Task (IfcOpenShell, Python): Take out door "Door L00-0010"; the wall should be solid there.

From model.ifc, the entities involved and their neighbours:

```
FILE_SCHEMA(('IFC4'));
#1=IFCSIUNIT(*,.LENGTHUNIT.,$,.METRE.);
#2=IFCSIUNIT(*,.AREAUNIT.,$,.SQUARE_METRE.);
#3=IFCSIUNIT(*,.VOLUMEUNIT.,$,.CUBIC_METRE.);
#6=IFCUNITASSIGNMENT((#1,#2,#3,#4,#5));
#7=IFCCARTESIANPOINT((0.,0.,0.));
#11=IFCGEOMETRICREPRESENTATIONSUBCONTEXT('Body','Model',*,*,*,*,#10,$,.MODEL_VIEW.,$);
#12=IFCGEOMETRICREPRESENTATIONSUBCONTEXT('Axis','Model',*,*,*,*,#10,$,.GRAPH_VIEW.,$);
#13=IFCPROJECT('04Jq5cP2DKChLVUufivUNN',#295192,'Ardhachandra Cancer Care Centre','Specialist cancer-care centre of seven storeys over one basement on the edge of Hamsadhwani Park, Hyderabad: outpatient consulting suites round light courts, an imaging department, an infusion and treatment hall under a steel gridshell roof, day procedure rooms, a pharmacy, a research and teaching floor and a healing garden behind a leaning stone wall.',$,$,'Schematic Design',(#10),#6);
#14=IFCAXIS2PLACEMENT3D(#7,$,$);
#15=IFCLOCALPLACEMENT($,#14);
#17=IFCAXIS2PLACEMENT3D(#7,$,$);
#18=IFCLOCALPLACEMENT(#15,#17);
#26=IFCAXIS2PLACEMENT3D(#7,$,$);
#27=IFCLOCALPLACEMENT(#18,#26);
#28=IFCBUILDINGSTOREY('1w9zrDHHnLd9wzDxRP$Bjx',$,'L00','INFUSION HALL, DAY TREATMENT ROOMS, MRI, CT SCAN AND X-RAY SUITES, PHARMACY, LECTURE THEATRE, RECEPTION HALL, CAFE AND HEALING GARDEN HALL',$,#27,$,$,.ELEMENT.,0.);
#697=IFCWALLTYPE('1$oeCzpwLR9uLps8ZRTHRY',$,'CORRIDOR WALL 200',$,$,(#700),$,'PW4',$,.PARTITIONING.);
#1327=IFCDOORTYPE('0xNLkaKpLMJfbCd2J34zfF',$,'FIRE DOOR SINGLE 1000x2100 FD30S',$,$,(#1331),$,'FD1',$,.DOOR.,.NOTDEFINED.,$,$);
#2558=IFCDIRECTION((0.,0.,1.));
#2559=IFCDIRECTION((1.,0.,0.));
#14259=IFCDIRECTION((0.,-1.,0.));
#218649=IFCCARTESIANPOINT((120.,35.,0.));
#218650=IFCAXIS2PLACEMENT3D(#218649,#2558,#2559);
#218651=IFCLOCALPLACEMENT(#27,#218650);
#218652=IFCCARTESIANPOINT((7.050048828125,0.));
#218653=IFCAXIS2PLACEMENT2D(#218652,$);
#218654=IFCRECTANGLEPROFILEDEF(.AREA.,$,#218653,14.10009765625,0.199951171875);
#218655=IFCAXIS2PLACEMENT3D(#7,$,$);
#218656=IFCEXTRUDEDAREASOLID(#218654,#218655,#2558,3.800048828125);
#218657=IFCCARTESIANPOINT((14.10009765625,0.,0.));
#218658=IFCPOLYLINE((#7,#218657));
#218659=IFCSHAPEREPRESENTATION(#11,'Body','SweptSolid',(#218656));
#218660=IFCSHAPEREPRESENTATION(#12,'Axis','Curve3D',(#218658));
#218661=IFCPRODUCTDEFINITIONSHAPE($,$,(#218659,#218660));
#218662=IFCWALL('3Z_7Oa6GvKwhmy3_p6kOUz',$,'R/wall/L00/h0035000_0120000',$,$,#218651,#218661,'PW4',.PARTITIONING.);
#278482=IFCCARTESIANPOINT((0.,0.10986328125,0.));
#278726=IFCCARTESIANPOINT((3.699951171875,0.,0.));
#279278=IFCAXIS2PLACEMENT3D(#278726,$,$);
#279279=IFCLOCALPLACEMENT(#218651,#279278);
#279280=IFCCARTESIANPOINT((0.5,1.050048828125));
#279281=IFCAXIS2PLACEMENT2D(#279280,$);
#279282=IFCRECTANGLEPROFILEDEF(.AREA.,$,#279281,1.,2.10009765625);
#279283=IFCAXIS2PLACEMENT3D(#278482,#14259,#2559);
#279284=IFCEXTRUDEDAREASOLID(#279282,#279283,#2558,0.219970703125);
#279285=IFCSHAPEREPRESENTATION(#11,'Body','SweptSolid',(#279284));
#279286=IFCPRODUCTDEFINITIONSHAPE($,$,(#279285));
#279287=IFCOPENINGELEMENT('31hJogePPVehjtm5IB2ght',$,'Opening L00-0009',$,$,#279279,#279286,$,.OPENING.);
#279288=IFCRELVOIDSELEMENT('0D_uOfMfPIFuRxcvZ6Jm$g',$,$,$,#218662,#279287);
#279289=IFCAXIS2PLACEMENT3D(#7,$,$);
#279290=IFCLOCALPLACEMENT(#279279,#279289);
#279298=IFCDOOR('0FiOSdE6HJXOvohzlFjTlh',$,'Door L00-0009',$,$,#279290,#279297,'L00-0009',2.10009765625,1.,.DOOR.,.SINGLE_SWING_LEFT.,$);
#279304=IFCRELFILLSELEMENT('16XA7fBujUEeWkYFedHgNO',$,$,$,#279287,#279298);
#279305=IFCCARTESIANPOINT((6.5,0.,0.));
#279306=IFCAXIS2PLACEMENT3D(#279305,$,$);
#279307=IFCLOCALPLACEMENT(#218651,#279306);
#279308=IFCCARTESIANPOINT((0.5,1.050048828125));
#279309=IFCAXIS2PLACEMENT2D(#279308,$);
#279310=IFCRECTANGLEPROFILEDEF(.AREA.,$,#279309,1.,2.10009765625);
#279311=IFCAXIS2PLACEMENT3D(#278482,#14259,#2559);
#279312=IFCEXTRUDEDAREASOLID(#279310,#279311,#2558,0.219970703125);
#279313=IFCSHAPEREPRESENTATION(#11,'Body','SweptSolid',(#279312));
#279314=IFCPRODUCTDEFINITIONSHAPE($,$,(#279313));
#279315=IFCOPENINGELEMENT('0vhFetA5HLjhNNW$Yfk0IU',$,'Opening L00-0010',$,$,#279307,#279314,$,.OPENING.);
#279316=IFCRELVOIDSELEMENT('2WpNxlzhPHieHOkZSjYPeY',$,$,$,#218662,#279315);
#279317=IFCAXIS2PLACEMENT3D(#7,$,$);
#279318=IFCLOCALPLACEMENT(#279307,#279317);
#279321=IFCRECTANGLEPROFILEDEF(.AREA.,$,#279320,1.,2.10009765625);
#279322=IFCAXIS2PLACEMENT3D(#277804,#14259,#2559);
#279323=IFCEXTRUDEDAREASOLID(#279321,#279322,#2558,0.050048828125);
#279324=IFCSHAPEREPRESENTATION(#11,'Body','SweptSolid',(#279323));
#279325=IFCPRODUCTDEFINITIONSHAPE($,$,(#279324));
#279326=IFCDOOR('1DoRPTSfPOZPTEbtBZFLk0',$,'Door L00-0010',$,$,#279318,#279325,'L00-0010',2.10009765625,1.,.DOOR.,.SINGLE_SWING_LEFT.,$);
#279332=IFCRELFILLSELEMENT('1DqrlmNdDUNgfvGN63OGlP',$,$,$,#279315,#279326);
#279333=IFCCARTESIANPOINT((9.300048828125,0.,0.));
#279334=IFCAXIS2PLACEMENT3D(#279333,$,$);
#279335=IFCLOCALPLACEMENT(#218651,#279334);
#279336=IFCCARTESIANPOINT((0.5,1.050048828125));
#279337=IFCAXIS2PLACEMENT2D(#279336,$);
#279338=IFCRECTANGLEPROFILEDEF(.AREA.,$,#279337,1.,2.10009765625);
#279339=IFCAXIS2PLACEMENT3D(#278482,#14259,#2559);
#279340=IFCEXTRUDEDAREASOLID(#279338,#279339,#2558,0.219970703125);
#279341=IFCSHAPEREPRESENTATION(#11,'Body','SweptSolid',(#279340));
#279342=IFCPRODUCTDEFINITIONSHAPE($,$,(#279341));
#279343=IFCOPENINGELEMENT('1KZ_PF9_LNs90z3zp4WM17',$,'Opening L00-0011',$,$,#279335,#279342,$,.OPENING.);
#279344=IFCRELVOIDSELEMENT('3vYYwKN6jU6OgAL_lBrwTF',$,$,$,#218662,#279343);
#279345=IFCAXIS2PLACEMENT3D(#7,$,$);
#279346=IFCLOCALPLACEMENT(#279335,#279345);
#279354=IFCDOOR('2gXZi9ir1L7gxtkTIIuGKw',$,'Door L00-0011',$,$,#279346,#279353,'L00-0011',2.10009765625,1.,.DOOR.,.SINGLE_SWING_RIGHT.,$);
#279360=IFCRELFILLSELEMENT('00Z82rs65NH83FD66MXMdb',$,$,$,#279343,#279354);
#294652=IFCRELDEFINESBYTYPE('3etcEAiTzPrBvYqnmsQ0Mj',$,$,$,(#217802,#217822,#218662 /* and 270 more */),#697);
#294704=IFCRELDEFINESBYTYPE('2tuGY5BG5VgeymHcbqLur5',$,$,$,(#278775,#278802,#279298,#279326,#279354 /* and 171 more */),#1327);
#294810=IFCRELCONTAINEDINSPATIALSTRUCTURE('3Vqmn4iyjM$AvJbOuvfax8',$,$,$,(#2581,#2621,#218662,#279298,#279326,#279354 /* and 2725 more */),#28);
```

```python
import ifcopenshell
import ifcopenshell.api.feature
import ifcopenshell.api.root
import ifcopenshell.geom
import ifcopenshell.util.shape

model = ifcopenshell.open("model.ifc")
settings = ifcopenshell.geom.settings()


def volume(element):
    """Net volume in cubic metres, openings subtracted."""
    shape = ifcopenshell.geom.create_shape(settings, element)
    return ifcopenshell.util.shape.get_volume(shape.geometry)


door = model.by_guid("1DoRPTSfPOZPTEbtBZFLk0")
opening = door.FillsVoids[0].RelatingOpeningElement
wall = opening.VoidsElements[0].RelatingBuildingElement
before = volume(wall)

ifcopenshell.api.root.remove_product(model, product=door)
ifcopenshell.api.feature.remove_feature(model, feature=opening)

after = volume(wall)

print(f"wall volume {before:.3f} -> {after:.3f} m3")

model.write("model_updated.ifc")
```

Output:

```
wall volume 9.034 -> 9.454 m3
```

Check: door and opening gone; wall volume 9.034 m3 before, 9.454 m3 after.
